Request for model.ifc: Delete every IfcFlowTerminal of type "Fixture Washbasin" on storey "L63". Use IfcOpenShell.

First a look at what the model holds.

```python
import ifcopenshell
import ifcopenshell.util.element

model = ifcopenshell.open("model.ifc")
print(model.schema)
storey = next(s for s in model.by_type("IfcBuildingStorey") if s.Name == "L63")
terminals = [e for e in ifcopenshell.util.element.get_decomposition(storey) if e.is_a("IfcFlowTerminal")]
seen = {}
for e in terminals:
    element_type = ifcopenshell.util.element.get_type(e)
    name = element_type.Name if element_type not in (None, e) else None
    seen[name] = seen.get(name, 0) + 1
for name, count in sorted(seen.items(), key=str):
    print(count, "x", name)
```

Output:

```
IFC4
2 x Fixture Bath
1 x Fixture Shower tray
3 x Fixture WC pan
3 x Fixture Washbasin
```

```python
import ifcopenshell
import ifcopenshell.api.root
import ifcopenshell.util.element

model = ifcopenshell.open("model.ifc")

storey = next(s for s in model.by_type("IfcBuildingStorey") if s.Name == "L63")
terminals = [e for e in ifcopenshell.util.element.get_decomposition(storey) if e.is_a("IfcFlowTerminal")]
targets = [e for e in terminals if (t := ifcopenshell.util.element.get_type(e)) not in (None, e) and t.Name == "Fixture Washbasin"]

for e in targets:
    ifcopenshell.api.root.remove_product(model, product=e)
print(len(targets), "removed")

model.write("model_rev.ifc")
```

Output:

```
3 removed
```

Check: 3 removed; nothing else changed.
